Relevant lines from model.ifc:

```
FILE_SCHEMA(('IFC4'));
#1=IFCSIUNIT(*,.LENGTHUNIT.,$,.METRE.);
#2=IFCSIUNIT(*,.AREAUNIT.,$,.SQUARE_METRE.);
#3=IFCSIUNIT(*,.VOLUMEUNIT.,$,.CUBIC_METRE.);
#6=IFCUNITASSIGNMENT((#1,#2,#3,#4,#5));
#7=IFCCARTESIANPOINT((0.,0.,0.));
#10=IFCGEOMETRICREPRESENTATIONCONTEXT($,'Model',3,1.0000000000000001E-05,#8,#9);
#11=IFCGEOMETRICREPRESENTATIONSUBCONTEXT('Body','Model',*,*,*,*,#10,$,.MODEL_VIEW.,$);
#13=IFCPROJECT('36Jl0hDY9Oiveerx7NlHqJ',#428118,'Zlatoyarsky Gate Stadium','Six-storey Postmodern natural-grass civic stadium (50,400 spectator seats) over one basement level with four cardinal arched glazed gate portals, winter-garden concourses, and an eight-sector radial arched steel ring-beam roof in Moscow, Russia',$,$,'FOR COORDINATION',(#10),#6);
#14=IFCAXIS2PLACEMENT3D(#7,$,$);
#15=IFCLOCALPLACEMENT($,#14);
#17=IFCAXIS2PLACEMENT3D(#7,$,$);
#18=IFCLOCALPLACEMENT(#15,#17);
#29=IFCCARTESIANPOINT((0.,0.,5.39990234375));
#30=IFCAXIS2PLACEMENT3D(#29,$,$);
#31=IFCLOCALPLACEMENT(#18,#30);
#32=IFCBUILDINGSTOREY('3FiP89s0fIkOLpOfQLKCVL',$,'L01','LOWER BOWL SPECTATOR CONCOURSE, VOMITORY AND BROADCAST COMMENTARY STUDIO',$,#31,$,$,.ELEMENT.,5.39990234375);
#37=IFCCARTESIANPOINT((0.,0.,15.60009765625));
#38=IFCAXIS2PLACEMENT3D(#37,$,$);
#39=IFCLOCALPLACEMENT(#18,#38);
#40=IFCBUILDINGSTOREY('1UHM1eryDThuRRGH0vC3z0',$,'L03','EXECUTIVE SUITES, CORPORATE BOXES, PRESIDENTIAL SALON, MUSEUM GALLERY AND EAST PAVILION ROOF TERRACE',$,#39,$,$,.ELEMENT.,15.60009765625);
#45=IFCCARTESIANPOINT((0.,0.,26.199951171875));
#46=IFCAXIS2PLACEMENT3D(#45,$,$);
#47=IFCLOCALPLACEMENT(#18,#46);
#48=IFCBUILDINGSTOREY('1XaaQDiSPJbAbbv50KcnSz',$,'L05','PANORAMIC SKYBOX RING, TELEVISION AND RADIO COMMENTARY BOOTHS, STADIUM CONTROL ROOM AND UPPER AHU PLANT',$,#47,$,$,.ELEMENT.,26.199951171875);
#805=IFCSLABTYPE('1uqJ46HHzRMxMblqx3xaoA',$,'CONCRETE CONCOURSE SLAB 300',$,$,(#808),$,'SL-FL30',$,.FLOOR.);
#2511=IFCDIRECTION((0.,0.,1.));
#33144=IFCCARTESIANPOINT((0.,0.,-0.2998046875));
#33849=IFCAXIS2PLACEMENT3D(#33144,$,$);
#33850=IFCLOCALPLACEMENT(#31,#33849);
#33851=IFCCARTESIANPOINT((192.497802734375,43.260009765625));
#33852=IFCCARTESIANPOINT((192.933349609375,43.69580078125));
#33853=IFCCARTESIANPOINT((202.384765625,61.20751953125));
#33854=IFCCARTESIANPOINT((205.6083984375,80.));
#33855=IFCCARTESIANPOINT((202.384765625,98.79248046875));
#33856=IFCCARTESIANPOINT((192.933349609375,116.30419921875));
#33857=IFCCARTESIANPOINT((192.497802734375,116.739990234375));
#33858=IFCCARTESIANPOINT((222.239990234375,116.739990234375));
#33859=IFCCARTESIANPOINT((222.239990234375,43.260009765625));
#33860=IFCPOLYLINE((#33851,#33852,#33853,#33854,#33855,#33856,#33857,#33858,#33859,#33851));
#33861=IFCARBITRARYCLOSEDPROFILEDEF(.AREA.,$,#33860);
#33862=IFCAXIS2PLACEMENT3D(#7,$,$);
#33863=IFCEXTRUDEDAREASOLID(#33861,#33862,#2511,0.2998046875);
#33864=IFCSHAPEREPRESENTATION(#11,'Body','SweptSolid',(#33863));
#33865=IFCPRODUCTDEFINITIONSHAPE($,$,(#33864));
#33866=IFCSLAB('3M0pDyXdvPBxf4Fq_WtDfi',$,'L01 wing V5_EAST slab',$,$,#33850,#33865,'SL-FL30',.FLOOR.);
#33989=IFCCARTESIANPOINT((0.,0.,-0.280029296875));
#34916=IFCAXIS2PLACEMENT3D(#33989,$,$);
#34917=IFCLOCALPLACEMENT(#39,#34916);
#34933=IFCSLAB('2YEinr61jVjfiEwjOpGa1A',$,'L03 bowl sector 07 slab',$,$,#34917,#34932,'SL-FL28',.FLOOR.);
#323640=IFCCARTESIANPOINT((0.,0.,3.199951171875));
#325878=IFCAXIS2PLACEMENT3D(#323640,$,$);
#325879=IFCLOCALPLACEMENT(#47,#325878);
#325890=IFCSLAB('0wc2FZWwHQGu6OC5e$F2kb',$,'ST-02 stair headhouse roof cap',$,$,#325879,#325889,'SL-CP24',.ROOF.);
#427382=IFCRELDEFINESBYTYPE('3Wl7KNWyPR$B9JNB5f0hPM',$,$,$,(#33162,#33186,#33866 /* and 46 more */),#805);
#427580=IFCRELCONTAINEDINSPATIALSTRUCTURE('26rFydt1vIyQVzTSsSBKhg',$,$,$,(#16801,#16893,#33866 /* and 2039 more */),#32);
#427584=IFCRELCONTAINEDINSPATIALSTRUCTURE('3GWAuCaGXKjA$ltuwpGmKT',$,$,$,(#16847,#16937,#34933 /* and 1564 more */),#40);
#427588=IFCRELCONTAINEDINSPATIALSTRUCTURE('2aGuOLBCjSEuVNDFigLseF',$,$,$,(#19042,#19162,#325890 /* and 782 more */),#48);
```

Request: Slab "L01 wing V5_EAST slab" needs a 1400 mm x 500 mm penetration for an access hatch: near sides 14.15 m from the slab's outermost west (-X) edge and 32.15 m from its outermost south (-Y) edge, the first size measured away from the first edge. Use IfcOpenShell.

```python
import numpy as np
import ifcopenshell
import ifcopenshell.api.feature
import ifcopenshell.api.geometry
import ifcopenshell.api.root
import ifcopenshell.geom
import ifcopenshell.util.placement
import ifcopenshell.util.representation
import ifcopenshell.util.shape
import ifcopenshell.util.unit

model = ifcopenshell.open("model.ifc")
unit_scale = ifcopenshell.util.unit.calculate_unit_scale(model)
settings = ifcopenshell.geom.settings()


def volume(element):
    """Net volume in cubic metres, openings subtracted."""
    shape = ifcopenshell.geom.create_shape(settings, element)
    return ifcopenshell.util.shape.get_volume(shape.geometry)


slab = model.by_guid("3M0pDyXdvPBxf4Fq_WtDfi")
before = volume(slab)

# Extent in the slab's own axes, in metres. The edges named are its -X and -Y sides.
slab_shape = ifcopenshell.geom.create_shape(settings, slab)
vertices = ifcopenshell.util.shape.get_vertices(slab_shape.geometry)
x_min, y_min, bottom = vertices.min(axis=0)
top = vertices[:, 2].max()

opening = ifcopenshell.api.root.create_entity(model, ifc_class="IfcOpeningElement", name="Access hatch opening", predefined_type="OPENING")
context = ifcopenshell.util.representation.get_context(model, "Model", "Body", "MODEL_VIEW")
width, depth = 1.4, 0.5
outline = [(0.0, 0.0), (width, 0.0), (width, depth), (0.0, depth), (0.0, 0.0)]
# Overshoot both faces by 50 mm so the cut is clean.
shape = ifcopenshell.api.geometry.add_slab_representation(
    model, context=context, depth=top - bottom + 0.1, polyline=outline
)
ifcopenshell.api.geometry.assign_representation(model, product=opening, representation=shape)

matrix = ifcopenshell.util.placement.get_local_placement(slab.ObjectPlacement)
matrix[:, 3] = matrix @ np.append(np.array([x_min + 14.15, y_min + 32.15, bottom - 0.05]) / unit_scale, 1.0)
ifcopenshell.api.geometry.edit_object_placement(model, product=opening, matrix=matrix, is_si=False)
ifcopenshell.api.feature.add_feature(model, feature=opening, element=slab)

after = volume(slab)

print(f"slab volume {before:.3f} -> {after:.3f} m3")

model.write("model_updated.ifc")
```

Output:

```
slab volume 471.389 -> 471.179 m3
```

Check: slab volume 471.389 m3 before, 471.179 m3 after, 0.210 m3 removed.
